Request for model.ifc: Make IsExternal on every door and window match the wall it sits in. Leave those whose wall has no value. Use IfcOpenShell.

First a look at what the model holds.

```python
import ifcopenshell
import ifcopenshell.util.element

model = ifcopenshell.open("model.ifc")
print(model.schema)
seen = {}
for e in model.by_type("IfcDoor") + model.by_type("IfcWindow"):
    if not e.FillsVoids:
        continue
    host = e.FillsVoids[0].RelatingOpeningElement.VoidsElements[0].RelatingBuildingElement
    own = ifcopenshell.util.element.get_pset(e, f"Pset_{e.is_a()[3:].removesuffix('StandardCase')}Common", "IsExternal")
    wall = ifcopenshell.util.element.get_pset(host, "Pset_WallCommon", "IsExternal")
    seen[e.is_a(), own, wall] = seen.get((e.is_a(), own, wall), 0) + 1
for (cls, own, wall), count in sorted(seen.items(), key=str):
    print(count, cls, "IsExternal:", own, "| host wall:", wall)
```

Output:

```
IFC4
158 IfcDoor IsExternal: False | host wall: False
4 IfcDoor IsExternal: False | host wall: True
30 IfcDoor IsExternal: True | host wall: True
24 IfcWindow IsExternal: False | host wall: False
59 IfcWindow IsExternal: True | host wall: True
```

```python
import ifcopenshell
import ifcopenshell.api.pset
import ifcopenshell.util.element

model = ifcopenshell.open("model.ifc")

count = 0
for ifc_class, pset_name in (("IfcDoor", "Pset_DoorCommon"), ("IfcWindow", "Pset_WindowCommon")):
    for e in model.by_type(ifc_class):
        if not e.FillsVoids:
            continue
        host = e.FillsVoids[0].RelatingOpeningElement.VoidsElements[0].RelatingBuildingElement
        external = ifcopenshell.util.element.get_pset(host, "Pset_WallCommon", "IsExternal")
        if external is None or ifcopenshell.util.element.get_pset(e, pset_name, "IsExternal") == external:
            continue
        pset = ifcopenshell.api.pset.add_pset(model, product=e, name=pset_name)
        ifcopenshell.api.pset.edit_pset(model, pset=pset, properties={"IsExternal": external})
        count += 1

print(count, "updated")

model.write("model_edited.ifc")
```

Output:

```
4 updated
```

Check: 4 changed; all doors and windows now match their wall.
